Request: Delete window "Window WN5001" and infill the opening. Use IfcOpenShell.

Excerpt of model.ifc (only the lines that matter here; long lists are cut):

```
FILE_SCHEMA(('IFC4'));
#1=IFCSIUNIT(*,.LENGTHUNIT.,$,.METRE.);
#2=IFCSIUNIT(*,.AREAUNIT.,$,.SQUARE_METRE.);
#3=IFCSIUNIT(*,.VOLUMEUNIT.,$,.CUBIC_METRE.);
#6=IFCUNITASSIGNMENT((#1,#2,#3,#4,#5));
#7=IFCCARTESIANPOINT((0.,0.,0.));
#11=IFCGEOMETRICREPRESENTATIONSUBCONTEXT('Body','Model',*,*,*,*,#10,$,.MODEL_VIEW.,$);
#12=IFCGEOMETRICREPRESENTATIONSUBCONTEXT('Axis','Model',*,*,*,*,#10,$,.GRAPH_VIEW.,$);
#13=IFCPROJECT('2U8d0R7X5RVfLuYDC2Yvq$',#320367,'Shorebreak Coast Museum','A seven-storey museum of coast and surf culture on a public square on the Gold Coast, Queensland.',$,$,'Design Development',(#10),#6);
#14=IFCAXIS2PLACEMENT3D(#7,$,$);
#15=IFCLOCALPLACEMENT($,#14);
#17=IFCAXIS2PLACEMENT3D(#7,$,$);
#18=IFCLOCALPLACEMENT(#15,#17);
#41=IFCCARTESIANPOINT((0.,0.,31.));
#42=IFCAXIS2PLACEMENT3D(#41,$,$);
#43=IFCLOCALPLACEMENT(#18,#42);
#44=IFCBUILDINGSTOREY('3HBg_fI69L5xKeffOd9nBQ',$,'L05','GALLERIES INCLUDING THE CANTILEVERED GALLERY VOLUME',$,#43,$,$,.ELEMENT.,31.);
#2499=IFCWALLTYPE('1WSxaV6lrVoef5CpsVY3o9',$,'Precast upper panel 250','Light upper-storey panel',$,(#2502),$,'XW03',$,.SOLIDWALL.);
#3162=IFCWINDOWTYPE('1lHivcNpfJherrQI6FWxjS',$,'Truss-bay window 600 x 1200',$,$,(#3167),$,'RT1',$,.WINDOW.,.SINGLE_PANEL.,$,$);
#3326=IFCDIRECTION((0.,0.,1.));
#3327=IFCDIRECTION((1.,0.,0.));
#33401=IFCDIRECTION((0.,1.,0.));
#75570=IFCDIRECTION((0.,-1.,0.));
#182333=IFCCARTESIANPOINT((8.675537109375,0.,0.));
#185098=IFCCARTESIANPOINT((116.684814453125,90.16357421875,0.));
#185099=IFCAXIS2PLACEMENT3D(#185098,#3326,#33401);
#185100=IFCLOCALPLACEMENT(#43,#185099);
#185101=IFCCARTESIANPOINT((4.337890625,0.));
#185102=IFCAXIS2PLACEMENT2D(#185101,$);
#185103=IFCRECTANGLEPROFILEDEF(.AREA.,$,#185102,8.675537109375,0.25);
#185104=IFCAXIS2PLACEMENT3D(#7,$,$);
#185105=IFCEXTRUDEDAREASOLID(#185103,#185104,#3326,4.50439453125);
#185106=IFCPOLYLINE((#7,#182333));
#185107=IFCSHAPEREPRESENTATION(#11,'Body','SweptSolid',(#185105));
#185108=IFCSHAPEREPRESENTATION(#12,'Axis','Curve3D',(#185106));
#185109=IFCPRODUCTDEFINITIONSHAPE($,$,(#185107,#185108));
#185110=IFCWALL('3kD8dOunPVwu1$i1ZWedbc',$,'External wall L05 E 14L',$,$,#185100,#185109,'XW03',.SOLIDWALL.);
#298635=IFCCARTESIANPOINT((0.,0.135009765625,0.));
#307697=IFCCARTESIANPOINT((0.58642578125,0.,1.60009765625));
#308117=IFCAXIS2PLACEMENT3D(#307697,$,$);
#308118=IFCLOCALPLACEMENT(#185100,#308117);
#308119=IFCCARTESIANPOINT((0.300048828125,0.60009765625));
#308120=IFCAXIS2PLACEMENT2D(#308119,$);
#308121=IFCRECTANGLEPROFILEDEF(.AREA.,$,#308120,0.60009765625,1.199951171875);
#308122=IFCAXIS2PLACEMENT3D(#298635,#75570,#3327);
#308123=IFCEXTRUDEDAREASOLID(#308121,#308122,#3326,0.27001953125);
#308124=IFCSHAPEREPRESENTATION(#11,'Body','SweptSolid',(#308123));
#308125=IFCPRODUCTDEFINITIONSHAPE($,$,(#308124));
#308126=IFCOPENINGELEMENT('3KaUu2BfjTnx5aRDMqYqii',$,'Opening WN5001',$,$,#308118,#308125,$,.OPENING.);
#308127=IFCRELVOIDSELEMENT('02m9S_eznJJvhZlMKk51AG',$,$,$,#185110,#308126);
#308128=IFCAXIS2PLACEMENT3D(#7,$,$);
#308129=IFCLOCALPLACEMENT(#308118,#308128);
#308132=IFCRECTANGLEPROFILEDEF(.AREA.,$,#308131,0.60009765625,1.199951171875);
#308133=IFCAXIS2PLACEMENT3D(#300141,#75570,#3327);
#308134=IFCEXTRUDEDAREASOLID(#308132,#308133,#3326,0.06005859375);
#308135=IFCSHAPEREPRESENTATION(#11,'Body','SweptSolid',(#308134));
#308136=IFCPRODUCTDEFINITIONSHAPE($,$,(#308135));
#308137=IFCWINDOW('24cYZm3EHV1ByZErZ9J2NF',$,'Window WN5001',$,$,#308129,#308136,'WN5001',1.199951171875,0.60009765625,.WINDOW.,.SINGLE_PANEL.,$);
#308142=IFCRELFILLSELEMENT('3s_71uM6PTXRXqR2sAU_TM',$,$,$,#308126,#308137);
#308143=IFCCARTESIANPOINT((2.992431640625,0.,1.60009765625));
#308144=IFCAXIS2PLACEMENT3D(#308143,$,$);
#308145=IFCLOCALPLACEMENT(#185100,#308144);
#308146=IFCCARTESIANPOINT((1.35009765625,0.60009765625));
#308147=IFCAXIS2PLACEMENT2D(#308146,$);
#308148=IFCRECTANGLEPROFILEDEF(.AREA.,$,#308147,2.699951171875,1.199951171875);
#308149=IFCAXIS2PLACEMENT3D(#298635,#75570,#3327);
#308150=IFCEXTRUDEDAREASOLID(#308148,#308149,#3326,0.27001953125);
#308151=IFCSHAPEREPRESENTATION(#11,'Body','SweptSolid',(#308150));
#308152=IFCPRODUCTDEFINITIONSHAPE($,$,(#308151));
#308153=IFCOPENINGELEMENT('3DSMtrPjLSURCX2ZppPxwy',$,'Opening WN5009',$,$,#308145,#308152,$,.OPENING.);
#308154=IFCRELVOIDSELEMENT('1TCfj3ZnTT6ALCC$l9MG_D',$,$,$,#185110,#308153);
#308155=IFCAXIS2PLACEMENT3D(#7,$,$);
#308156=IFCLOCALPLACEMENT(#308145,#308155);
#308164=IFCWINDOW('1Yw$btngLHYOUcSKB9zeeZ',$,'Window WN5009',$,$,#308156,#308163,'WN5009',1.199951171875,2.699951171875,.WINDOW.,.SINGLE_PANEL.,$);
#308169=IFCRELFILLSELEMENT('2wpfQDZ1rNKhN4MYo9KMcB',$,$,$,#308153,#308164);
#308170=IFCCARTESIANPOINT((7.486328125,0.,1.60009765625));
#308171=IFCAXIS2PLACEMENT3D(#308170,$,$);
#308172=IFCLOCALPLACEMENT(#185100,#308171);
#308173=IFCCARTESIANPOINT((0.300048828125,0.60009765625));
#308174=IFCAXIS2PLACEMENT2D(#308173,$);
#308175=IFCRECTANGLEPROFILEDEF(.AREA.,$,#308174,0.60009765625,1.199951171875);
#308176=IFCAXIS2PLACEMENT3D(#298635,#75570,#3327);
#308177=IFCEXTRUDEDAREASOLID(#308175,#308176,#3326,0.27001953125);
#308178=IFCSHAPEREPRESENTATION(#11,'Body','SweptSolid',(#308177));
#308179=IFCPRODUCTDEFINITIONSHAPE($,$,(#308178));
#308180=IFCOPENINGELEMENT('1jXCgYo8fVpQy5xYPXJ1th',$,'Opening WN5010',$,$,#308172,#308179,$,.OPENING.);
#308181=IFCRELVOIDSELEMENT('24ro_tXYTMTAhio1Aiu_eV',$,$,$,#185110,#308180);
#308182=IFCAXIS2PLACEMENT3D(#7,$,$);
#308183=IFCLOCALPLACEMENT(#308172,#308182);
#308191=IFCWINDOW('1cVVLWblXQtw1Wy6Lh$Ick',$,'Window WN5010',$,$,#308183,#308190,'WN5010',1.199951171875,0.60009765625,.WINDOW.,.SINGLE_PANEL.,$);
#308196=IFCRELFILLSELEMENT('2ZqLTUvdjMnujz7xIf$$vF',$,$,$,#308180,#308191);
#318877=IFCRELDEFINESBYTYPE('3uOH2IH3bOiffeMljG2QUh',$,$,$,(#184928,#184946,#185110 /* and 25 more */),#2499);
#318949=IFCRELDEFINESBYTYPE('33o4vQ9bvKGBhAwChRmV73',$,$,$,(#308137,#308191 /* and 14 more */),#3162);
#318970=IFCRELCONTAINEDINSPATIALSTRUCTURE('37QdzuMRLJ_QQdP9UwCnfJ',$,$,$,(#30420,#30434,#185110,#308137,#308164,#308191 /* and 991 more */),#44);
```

```python
import ifcopenshell
import ifcopenshell.api.feature
import ifcopenshell.api.root
import ifcopenshell.geom
import ifcopenshell.util.shape

model = ifcopenshell.open("model.ifc")
settings = ifcopenshell.geom.settings()


def volume(element):
    """Net volume in cubic metres, openings subtracted."""
    shape = ifcopenshell.geom.create_shape(settings, element)
    return ifcopenshell.util.shape.get_volume(shape.geometry)


window = model.by_guid("24cYZm3EHV1ByZErZ9J2NF")
opening = window.FillsVoids[0].RelatingOpeningElement
wall = opening.VoidsElements[0].RelatingBuildingElement
before = volume(wall)

ifcopenshell.api.root.remove_product(model, product=window)
ifcopenshell.api.feature.remove_feature(model, feature=opening)

after = volume(wall)

print(f"wall volume {before:.3f} -> {after:.3f} m3")

model.write("model_rev.ifc")
```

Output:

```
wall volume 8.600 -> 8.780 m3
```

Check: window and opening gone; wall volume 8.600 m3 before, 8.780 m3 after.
